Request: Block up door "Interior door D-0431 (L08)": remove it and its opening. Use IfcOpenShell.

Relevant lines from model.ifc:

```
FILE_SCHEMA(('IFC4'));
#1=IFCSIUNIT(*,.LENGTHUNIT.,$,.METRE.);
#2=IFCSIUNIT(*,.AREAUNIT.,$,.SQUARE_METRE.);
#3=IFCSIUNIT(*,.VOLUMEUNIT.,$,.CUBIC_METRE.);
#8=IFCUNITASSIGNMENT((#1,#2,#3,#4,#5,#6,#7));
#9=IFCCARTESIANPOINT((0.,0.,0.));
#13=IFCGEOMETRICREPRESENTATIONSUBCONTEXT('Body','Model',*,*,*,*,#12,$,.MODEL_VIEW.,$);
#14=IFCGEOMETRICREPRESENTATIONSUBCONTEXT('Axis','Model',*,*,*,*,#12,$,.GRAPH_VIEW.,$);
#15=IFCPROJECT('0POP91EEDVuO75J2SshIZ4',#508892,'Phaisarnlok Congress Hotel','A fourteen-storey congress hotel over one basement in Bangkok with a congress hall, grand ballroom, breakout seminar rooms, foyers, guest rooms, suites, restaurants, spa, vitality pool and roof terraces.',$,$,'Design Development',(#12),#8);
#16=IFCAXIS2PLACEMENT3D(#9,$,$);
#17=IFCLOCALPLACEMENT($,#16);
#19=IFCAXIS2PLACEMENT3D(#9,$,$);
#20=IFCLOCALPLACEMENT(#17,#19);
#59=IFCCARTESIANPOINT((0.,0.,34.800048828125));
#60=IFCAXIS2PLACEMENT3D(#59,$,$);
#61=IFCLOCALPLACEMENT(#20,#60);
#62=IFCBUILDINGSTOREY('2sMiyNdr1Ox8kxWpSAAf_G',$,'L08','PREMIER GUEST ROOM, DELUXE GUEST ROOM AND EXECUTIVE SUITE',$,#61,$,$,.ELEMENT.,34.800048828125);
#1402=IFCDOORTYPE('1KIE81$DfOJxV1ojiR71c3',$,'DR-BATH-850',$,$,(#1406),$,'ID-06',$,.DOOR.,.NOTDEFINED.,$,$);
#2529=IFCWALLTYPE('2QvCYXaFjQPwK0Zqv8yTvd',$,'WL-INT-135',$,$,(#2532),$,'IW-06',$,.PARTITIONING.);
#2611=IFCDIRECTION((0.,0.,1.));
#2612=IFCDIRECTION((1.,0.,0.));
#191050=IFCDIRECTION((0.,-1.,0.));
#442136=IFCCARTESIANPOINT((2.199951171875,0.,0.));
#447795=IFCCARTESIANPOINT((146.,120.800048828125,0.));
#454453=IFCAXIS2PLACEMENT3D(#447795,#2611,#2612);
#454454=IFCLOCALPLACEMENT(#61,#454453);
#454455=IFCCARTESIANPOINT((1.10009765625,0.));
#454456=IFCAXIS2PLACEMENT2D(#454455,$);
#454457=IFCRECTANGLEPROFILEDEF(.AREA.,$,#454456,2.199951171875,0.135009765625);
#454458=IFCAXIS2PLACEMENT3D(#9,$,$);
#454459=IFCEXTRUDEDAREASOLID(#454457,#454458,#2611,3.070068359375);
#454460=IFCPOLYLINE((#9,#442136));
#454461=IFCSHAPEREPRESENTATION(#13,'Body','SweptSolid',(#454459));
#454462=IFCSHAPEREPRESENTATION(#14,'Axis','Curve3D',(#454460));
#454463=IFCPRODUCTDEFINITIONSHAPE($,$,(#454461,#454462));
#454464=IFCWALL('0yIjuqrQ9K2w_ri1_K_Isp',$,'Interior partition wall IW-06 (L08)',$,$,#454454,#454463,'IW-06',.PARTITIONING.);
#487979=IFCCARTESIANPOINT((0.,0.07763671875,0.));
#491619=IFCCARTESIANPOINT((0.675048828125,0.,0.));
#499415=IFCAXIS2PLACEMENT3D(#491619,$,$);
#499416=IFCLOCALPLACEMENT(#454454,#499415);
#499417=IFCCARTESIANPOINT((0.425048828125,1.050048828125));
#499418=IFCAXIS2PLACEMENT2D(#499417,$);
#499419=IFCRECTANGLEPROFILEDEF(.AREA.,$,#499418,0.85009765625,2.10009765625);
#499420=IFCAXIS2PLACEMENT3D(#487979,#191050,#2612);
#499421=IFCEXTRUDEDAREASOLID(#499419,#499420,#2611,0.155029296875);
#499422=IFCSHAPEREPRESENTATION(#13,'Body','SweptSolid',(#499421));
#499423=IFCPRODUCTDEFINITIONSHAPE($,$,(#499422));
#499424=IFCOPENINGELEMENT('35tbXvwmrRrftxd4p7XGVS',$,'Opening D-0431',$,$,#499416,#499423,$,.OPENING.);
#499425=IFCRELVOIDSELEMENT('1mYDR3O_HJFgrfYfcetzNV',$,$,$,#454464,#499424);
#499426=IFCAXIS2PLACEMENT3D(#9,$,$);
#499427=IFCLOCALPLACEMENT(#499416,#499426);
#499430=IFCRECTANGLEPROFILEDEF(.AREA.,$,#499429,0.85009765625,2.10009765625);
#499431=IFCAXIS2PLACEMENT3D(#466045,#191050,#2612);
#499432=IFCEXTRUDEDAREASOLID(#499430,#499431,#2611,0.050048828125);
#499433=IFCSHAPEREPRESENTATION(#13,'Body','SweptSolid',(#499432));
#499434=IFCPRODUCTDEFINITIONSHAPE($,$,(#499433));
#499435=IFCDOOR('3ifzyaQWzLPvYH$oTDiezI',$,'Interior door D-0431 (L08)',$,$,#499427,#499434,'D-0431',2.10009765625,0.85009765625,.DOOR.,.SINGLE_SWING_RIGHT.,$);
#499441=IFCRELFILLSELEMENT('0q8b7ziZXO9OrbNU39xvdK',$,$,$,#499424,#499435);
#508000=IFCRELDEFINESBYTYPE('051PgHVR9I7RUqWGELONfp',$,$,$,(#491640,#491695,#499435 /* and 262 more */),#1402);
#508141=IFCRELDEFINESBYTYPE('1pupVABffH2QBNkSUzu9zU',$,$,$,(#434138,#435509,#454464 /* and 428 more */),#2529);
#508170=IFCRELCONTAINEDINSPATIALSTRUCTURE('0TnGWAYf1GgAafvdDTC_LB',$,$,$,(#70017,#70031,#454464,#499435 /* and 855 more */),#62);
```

```python
import ifcopenshell
import ifcopenshell.api.feature
import ifcopenshell.api.root
import ifcopenshell.geom
import ifcopenshell.util.shape

model = ifcopenshell.open("model.ifc")
settings = ifcopenshell.geom.settings()


def volume(element):
    """Net volume in cubic metres, openings subtracted."""
    shape = ifcopenshell.geom.create_shape(settings, element)
    return ifcopenshell.util.shape.get_volume(shape.geometry)


door = model.by_guid("3ifzyaQWzLPvYH$oTDiezI")
opening = door.FillsVoids[0].RelatingOpeningElement
wall = opening.VoidsElements[0].RelatingBuildingElement
before = volume(wall)

ifcopenshell.api.root.remove_product(model, product=door)
ifcopenshell.api.feature.remove_feature(model, feature=opening)

after = volume(wall)

print(f"wall volume {before:.3f} -> {after:.3f} m3")

model.write("model_v2.ifc")
```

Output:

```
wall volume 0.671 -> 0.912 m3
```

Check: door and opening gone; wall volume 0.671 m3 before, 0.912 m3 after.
